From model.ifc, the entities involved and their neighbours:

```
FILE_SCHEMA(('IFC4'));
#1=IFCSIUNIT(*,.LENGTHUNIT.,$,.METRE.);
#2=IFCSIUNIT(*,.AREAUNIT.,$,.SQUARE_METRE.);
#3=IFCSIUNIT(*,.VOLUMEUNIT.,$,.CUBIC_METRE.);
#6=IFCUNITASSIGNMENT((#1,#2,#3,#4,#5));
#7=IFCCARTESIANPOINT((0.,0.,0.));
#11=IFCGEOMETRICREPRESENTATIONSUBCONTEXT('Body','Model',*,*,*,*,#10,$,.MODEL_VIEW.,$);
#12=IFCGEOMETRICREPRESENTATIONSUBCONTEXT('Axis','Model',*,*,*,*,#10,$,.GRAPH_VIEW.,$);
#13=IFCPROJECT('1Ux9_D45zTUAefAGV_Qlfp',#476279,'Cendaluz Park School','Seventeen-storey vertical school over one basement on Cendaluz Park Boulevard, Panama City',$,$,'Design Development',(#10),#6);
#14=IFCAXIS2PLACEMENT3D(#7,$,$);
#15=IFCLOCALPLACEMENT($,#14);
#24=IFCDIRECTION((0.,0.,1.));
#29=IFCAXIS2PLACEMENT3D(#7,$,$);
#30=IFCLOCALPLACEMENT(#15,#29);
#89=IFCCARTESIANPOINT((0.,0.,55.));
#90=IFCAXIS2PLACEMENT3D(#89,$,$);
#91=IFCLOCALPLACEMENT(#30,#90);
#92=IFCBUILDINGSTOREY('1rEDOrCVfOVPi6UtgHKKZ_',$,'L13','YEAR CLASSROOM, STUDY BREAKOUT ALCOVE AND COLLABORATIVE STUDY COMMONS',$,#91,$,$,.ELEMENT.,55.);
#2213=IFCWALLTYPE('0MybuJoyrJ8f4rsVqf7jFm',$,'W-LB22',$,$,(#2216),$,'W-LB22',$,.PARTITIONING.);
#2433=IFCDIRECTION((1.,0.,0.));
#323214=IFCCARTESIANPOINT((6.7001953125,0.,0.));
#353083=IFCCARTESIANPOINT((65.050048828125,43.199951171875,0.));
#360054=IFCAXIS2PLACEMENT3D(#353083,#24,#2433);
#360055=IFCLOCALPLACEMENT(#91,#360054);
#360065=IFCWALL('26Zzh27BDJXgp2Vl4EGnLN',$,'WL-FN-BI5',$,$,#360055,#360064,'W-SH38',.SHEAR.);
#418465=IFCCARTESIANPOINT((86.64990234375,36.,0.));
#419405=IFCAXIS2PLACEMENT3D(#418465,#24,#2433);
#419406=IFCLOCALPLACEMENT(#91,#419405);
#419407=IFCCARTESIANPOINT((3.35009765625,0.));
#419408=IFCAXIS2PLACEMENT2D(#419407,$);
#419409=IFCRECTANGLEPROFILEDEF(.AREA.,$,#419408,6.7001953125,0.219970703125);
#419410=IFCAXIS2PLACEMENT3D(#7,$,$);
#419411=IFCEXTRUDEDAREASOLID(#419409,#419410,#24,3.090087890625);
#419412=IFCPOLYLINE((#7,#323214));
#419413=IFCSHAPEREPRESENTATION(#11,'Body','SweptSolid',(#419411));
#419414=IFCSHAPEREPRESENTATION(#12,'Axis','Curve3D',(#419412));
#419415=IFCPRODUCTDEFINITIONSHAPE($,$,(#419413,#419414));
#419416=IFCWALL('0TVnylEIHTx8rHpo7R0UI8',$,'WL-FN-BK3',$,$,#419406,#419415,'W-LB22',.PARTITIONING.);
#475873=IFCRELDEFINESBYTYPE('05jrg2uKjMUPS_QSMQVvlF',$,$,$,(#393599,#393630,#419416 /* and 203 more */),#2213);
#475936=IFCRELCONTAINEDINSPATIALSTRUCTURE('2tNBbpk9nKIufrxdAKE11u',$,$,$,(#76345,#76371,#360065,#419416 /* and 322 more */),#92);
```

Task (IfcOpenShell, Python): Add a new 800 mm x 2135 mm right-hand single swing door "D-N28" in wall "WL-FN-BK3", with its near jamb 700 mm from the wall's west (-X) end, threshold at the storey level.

```python
import numpy as np
import ifcopenshell
import ifcopenshell.api.feature
import ifcopenshell.api.geometry
import ifcopenshell.api.root
import ifcopenshell.api.spatial
import ifcopenshell.geom
import ifcopenshell.util.element
import ifcopenshell.util.placement
import ifcopenshell.util.representation
import ifcopenshell.util.shape
import ifcopenshell.util.unit

model = ifcopenshell.open("model.ifc")
unit_scale = ifcopenshell.util.unit.calculate_unit_scale(model)
settings = ifcopenshell.geom.settings()


def volume(element):
    """Net volume in cubic metres, openings subtracted."""
    shape = ifcopenshell.geom.create_shape(settings, element)
    return ifcopenshell.util.shape.get_volume(shape.geometry)


wall = model.by_guid("0TVnylEIHTx8rHpo7R0UI8")
storey = ifcopenshell.util.element.get_container(wall, ifc_class="IfcBuildingStorey")
context = ifcopenshell.util.representation.get_context(model, "Model", "Body", "MODEL_VIEW")
before = volume(wall)

width, height, from_end, sill = 0.8, 2.135, 0.7, 0.0  # metres

# The wall runs along its own X axis, and the end named is its -X end.
wall_shape = ifcopenshell.geom.create_shape(settings, wall)
x, y, z = ifcopenshell.util.shape.get_vertices(wall_shape.geometry).T
start = x.min() + from_end
face, thickness = float(y.min()), float(y.max() - y.min())
wall_matrix = ifcopenshell.util.placement.get_local_placement(wall.ObjectPlacement)
level = ifcopenshell.util.placement.get_local_placement(storey.ObjectPlacement)[2, 3]


def in_wall(x, y):
    """Placement at x, y metres in the wall's axes, at sill height."""
    matrix = wall_matrix.copy()
    matrix[:, 3] = wall_matrix @ np.array([x / unit_scale, y / unit_scale, 0.0, 1.0])
    matrix[2, 3] = level + sill / unit_scale
    return matrix


# Opening: a box that overshoots both wall faces by 50 mm.
opening = ifcopenshell.api.root.create_entity(model, ifc_class="IfcOpeningElement", predefined_type="OPENING")
box = ifcopenshell.api.geometry.add_wall_representation(
    model, context=context, length=width, height=height, thickness=thickness + 0.1
)
ifcopenshell.api.geometry.assign_representation(model, product=opening, representation=box)
ifcopenshell.api.geometry.edit_object_placement(model, product=opening, matrix=in_wall(start, face - 0.05), is_si=False)
ifcopenshell.api.feature.add_feature(model, feature=opening, element=wall)

door = ifcopenshell.api.root.create_entity(model, ifc_class="IfcDoor", name="D-N28", predefined_type="DOOR")
door.OverallWidth, door.OverallHeight = width / unit_scale, height / unit_scale
door.OperationType = "SINGLE_SWING_RIGHT"
body = ifcopenshell.api.geometry.add_door_representation(
    model,
    context=context,
    overall_width=door.OverallWidth,
    overall_height=door.OverallHeight,
    operation_type="SINGLE_SWING_RIGHT",
    lining_properties={"LiningDepth": thickness / unit_scale, "ThresholdDepth": thickness / unit_scale},
)
ifcopenshell.api.geometry.assign_representation(model, product=door, representation=body)
ifcopenshell.api.spatial.assign_container(model, products=[door], relating_structure=storey)
ifcopenshell.api.feature.add_filling(model, opening=opening, element=door)

# The lining spans the wall, so the door starts at the wall face.
ifcopenshell.api.geometry.edit_object_placement(model, product=door, matrix=in_wall(start, face), is_si=False)

after = volume(wall)

print(f"wall volume {before:.3f} -> {after:.3f} m3")

model.write("model_updated.ifc")
```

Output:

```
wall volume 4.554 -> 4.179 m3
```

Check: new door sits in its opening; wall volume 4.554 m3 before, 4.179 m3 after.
